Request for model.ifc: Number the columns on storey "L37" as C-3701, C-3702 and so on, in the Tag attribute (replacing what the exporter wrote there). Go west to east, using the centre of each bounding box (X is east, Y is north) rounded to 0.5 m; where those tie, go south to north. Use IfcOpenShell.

First a look at what the model holds.

```python
import ifcopenshell
import ifcopenshell.util.element
import ifcopenshell.util.placement

model = ifcopenshell.open("model.ifc")
print(model.schema)
storey = next(s for s in model.by_type("IfcBuildingStorey") if s.Name == "L37")
columns = [e for e in ifcopenshell.util.element.get_decomposition(storey) if e.is_a("IfcColumn")]
for e in sorted(columns, key=lambda e: e.id()):
    origin = ifcopenshell.util.placement.get_local_placement(e.ObjectPlacement)[:3, 3]
    print(e.id(), e.Tag, e.Name, origin.round(2) + 0.0, sep=" | ")
```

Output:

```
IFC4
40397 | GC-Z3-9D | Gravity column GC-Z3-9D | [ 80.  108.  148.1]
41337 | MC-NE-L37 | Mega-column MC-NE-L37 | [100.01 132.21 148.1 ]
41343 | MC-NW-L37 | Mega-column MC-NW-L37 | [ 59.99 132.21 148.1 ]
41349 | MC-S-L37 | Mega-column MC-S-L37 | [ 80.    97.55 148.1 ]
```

```python
import ifcopenshell
import ifcopenshell.geom
import ifcopenshell.util.element
import ifcopenshell.util.shape

model = ifcopenshell.open("model.ifc")
settings = ifcopenshell.geom.settings()
settings.set("use-world-coords", True)


def centre(element):
    shape = ifcopenshell.geom.create_shape(settings, element)
    return ifcopenshell.util.shape.get_bbox_centroid(shape.geometry)


storey = next(s for s in model.by_type("IfcBuildingStorey") if s.Name == "L37")
columns = [e for e in ifcopenshell.util.element.get_decomposition(storey) if e.is_a("IfcColumn")]

# Insertion points can sit at a corner or the storey origin, so sort by the geometry (in metres).
centres = {e: centre(e) for e in columns}
columns.sort(key=lambda e: (round(centres[e][0] / 0.5), centres[e][1]))

for i, e in enumerate(columns, start=1):
    number = f"C-37{i:02d}"
    e.Tag = number
    print(e.id(), number)

model.write("model_v2.ifc")
```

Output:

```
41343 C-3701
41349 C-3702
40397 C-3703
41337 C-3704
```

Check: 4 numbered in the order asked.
